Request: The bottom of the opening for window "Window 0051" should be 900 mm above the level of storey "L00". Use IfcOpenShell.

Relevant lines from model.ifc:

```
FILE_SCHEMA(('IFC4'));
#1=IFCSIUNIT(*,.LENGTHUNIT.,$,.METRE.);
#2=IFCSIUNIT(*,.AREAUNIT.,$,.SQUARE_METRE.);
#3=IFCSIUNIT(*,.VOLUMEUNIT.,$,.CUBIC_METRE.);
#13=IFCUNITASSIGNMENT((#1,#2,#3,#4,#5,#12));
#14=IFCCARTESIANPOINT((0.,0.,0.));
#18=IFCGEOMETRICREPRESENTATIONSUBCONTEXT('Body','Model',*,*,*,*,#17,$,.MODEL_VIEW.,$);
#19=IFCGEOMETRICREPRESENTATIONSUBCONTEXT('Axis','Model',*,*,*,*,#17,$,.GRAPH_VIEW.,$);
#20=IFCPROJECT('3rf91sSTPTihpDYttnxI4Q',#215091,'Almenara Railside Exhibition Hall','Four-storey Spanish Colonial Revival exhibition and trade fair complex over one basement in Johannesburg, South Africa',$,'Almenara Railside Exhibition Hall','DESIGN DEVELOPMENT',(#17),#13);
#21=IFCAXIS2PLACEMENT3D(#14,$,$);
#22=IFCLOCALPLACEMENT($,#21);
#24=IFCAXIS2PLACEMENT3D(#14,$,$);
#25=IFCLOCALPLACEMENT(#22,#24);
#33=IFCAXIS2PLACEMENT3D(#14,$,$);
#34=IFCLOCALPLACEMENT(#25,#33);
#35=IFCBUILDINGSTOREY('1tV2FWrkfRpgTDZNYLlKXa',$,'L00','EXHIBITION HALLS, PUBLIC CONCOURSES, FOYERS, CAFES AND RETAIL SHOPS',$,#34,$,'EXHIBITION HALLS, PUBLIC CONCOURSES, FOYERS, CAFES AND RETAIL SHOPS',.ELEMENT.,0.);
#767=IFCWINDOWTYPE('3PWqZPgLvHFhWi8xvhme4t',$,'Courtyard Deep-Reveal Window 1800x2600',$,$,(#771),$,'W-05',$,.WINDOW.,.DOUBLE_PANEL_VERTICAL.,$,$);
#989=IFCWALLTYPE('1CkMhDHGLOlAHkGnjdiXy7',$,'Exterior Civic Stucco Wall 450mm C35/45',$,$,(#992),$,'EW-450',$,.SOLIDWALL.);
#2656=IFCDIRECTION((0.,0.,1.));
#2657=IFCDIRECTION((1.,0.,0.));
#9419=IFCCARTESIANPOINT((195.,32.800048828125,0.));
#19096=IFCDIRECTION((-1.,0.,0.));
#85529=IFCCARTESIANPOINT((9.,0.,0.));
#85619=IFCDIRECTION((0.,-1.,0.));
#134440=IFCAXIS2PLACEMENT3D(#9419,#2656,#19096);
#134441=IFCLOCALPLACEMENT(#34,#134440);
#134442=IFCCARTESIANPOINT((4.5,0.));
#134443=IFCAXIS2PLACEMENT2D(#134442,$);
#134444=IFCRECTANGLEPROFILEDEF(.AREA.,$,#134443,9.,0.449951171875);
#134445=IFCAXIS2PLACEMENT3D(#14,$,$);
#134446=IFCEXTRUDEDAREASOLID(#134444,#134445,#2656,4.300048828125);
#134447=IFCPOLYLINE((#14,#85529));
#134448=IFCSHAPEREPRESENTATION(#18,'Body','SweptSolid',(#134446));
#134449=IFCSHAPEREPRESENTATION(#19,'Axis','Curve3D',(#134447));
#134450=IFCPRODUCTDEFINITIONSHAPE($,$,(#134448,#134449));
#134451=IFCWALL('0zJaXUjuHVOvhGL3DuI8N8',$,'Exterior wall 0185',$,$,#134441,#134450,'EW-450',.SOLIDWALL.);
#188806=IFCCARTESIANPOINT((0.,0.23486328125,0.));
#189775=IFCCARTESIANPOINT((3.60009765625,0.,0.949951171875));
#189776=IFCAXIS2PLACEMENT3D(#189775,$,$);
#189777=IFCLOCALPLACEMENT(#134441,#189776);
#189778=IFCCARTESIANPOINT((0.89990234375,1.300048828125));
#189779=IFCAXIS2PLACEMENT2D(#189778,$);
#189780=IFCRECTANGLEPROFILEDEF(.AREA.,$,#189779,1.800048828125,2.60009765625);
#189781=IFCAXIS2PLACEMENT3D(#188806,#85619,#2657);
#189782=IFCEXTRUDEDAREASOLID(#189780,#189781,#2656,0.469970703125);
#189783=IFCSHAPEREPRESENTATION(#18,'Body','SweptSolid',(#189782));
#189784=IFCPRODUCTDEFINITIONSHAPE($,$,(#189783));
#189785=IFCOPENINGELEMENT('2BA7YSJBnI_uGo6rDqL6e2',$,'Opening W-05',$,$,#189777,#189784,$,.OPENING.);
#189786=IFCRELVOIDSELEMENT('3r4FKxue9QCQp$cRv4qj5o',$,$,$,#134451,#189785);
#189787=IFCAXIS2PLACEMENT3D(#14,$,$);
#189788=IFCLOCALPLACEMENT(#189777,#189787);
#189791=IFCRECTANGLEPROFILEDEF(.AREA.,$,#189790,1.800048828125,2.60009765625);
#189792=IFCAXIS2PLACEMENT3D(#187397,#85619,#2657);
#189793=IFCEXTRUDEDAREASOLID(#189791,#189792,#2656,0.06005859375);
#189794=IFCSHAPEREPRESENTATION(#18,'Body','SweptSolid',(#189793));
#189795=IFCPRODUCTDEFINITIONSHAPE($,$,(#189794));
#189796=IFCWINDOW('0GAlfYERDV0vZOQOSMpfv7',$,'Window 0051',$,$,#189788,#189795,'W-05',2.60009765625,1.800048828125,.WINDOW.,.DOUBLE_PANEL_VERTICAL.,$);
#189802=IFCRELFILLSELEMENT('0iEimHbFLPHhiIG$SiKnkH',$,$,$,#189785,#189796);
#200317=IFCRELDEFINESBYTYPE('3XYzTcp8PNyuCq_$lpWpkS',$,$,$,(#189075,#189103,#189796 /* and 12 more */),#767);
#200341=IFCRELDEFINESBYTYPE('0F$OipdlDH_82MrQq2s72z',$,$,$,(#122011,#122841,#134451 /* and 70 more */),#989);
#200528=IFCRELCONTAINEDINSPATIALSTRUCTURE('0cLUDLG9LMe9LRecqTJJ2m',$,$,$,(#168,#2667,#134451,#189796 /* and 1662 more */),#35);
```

```python
import numpy as np
import ifcopenshell
import ifcopenshell.api.geometry
import ifcopenshell.geom
import ifcopenshell.util.element
import ifcopenshell.util.placement
import ifcopenshell.util.shape
import ifcopenshell.util.unit

model = ifcopenshell.open("model.ifc")
unit_scale = ifcopenshell.util.unit.calculate_unit_scale(model)

window = model.by_id(189796)
opening = window.FillsVoids[0].RelatingOpeningElement
storey = ifcopenshell.util.element.get_container(window, ifc_class="IfcBuildingStorey")
level = ifcopenshell.util.placement.get_local_placement(storey.ObjectPlacement)[2, 3]

# The opening's origin need not be at the sill, so measure its lowest point.
shape = ifcopenshell.geom.create_shape(ifcopenshell.geom.settings(), opening)
bottom = ifcopenshell.util.shape.get_shape_bottom_elevation(shape, shape.geometry) / unit_scale
dz = level + 0.9 / unit_scale - bottom

shift = np.array([0.0, 0.0, dz])
# The window is placed relative to its opening, so it follows when the opening moves.
matrix = ifcopenshell.util.placement.get_local_placement(opening.ObjectPlacement)
matrix[:3, 3] += shift
ifcopenshell.api.geometry.edit_object_placement(
    model, product=opening, matrix=matrix, is_si=False, should_transform_children=True
)

print(f"moved by {dz * unit_scale:+.3f} m")

model.write("model_updated.ifc")
```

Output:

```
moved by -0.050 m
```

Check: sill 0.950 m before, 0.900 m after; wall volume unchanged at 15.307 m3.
